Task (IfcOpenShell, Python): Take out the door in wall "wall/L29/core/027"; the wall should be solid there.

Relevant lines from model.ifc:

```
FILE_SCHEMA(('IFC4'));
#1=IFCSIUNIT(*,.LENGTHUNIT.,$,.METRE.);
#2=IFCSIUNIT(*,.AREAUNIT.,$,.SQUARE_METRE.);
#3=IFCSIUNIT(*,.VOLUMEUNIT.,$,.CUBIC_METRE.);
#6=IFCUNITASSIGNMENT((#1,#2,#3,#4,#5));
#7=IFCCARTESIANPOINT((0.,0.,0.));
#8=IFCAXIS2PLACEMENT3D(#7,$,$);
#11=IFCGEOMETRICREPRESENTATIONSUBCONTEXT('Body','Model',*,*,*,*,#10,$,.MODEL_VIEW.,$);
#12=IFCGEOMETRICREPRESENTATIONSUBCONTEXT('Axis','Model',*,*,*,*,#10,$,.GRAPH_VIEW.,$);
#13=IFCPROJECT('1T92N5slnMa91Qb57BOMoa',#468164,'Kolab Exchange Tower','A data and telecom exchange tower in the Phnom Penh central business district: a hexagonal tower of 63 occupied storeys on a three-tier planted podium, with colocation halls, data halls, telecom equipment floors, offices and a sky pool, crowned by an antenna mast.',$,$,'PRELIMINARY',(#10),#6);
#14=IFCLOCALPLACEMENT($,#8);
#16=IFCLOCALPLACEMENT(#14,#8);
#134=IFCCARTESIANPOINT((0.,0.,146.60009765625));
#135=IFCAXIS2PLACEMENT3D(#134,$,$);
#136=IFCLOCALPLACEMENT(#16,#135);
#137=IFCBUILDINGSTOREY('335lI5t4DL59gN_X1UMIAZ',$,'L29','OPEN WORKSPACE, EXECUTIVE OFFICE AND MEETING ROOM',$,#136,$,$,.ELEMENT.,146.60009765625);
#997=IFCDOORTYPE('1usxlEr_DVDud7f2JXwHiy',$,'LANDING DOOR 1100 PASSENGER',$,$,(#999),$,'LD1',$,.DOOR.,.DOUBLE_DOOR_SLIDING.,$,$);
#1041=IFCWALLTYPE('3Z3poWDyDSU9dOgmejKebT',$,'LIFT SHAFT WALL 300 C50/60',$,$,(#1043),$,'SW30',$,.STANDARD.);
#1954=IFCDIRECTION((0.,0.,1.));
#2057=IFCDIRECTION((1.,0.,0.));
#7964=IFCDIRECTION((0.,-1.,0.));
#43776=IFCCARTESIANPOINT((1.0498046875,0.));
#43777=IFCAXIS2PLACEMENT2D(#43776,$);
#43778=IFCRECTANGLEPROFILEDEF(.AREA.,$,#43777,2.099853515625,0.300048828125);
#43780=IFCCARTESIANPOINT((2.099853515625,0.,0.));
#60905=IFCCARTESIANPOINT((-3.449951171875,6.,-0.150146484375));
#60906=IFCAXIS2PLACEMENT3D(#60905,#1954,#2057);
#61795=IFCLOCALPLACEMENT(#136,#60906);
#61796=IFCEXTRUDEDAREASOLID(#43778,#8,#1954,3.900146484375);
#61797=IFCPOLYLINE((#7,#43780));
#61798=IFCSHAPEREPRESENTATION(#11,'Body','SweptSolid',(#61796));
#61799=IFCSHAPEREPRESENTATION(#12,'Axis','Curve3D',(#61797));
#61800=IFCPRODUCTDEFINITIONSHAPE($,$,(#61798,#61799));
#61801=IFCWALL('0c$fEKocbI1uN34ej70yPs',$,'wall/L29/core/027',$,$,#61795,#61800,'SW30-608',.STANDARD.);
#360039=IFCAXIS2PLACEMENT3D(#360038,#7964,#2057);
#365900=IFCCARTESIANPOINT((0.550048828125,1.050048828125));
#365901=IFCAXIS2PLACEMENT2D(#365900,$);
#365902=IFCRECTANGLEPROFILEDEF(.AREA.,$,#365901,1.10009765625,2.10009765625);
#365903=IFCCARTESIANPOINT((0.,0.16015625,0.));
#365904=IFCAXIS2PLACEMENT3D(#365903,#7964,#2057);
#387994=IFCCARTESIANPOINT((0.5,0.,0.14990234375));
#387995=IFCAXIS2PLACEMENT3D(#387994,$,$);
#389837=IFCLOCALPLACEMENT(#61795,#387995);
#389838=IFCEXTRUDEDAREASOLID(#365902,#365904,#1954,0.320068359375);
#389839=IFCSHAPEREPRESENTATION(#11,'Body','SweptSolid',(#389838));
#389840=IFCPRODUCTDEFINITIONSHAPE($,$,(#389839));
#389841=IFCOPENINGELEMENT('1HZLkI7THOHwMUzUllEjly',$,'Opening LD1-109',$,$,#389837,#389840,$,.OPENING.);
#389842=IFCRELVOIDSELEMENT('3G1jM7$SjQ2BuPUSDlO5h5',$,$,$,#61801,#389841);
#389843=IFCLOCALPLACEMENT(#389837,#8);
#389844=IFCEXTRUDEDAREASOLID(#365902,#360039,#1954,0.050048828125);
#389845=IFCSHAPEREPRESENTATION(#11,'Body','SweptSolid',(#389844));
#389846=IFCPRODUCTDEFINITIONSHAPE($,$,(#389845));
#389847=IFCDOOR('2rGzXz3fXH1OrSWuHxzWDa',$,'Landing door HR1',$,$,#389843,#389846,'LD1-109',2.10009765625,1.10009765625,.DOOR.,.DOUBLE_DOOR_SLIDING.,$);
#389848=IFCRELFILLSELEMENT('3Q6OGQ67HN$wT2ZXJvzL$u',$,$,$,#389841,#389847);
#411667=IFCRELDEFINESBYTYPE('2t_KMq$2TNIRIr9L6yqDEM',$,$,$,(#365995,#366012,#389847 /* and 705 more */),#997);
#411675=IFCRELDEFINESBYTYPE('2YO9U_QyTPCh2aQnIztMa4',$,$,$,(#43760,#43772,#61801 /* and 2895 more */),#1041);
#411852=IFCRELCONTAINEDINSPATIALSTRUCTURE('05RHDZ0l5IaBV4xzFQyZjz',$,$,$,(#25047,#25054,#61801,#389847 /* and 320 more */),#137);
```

```python
import ifcopenshell
import ifcopenshell.api.feature
import ifcopenshell.api.root
import ifcopenshell.geom
import ifcopenshell.util.shape

model = ifcopenshell.open("model.ifc")
settings = ifcopenshell.geom.settings()


def volume(element):
    """Net volume in cubic metres, openings subtracted."""
    shape = ifcopenshell.geom.create_shape(settings, element)
    return ifcopenshell.util.shape.get_volume(shape.geometry)


door = model.by_guid("2rGzXz3fXH1OrSWuHxzWDa")
opening = door.FillsVoids[0].RelatingOpeningElement
wall = opening.VoidsElements[0].RelatingBuildingElement
before = volume(wall)

ifcopenshell.api.root.remove_product(model, product=door)
ifcopenshell.api.feature.remove_feature(model, feature=opening)

after = volume(wall)

print(f"wall volume {before:.3f} -> {after:.3f} m3")

model.write("model_edited.ifc")
```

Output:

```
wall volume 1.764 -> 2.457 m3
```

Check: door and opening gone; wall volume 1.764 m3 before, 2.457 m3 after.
